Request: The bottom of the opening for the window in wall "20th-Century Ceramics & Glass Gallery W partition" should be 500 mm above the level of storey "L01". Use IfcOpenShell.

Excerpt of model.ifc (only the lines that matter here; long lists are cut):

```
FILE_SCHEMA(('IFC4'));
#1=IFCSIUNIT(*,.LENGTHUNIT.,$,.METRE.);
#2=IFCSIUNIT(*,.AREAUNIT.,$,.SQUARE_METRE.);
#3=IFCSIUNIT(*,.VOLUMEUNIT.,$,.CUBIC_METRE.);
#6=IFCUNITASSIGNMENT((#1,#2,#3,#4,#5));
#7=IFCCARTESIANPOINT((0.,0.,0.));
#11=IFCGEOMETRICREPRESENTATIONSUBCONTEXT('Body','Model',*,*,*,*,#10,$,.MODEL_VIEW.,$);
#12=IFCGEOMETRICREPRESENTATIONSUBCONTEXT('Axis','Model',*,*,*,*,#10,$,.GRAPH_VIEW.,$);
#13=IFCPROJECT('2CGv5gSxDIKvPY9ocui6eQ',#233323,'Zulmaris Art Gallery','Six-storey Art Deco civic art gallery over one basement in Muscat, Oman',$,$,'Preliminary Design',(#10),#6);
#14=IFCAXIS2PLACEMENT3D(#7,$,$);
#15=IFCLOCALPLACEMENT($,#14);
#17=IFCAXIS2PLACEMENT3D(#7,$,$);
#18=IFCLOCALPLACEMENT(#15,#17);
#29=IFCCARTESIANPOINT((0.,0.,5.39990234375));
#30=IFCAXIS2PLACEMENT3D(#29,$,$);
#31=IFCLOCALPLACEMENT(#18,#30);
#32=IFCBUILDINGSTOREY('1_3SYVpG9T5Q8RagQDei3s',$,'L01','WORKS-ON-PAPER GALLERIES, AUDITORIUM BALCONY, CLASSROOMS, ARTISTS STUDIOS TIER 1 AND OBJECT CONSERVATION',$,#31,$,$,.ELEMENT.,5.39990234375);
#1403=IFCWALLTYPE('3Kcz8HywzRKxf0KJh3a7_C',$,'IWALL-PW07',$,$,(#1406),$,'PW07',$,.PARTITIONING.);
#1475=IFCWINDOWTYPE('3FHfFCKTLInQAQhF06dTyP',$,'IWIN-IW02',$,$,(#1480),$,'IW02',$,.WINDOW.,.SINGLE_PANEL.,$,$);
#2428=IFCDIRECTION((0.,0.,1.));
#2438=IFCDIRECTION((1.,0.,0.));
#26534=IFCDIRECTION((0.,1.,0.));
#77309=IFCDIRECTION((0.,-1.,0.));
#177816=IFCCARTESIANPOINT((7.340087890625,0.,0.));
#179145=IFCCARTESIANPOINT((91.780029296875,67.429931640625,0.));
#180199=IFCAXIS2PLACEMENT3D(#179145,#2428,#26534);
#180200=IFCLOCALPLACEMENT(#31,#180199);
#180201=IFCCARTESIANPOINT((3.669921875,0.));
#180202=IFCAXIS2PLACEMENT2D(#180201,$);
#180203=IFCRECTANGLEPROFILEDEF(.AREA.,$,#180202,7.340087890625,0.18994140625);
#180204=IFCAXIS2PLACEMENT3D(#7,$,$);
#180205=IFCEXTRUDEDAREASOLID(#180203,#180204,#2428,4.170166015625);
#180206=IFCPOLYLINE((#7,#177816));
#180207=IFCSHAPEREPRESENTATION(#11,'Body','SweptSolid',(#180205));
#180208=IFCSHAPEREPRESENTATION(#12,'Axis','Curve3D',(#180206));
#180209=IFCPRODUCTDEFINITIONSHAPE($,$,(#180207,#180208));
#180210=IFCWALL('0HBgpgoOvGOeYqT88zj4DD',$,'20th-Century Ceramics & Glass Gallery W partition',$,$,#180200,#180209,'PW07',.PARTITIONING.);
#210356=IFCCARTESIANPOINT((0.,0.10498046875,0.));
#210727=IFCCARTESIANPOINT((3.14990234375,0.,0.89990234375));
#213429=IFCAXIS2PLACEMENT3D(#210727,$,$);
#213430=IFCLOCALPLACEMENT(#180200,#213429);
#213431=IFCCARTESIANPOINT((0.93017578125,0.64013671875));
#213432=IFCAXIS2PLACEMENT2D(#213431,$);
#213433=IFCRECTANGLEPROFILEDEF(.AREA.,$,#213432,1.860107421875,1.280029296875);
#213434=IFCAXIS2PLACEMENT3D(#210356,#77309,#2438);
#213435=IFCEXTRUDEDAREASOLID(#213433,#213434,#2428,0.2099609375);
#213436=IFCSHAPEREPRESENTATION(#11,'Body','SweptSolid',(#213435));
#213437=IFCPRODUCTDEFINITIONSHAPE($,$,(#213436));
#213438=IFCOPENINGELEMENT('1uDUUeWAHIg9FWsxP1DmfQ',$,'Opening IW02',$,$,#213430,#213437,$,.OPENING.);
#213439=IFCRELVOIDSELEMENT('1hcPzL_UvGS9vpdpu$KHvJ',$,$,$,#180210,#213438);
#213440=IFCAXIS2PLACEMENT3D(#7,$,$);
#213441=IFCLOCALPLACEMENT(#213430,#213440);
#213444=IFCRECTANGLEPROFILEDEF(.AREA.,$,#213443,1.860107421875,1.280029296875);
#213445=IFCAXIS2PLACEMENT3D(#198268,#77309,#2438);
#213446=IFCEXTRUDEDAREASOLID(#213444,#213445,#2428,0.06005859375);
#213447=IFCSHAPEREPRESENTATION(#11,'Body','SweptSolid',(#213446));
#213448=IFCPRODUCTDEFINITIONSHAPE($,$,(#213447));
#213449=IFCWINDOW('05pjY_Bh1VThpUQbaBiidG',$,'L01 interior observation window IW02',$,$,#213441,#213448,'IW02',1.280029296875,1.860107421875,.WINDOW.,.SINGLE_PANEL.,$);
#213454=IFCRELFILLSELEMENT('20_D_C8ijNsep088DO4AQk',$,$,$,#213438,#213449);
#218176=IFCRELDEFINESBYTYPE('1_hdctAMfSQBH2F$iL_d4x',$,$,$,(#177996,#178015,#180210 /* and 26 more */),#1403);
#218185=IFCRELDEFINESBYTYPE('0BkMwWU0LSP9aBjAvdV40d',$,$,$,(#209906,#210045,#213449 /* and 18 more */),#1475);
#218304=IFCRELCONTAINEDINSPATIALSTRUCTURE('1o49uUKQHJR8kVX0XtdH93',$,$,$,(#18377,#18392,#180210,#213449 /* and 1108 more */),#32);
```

```python
import numpy as np
import ifcopenshell
import ifcopenshell.api.geometry
import ifcopenshell.geom
import ifcopenshell.util.element
import ifcopenshell.util.placement
import ifcopenshell.util.shape
import ifcopenshell.util.unit

model = ifcopenshell.open("model.ifc")
unit_scale = ifcopenshell.util.unit.calculate_unit_scale(model)

window = model.by_guid("05pjY_Bh1VThpUQbaBiidG")
opening = window.FillsVoids[0].RelatingOpeningElement
storey = ifcopenshell.util.element.get_container(window, ifc_class="IfcBuildingStorey")
level = ifcopenshell.util.placement.get_local_placement(storey.ObjectPlacement)[2, 3]

# The opening's origin need not be at the sill, so measure its lowest point.
shape = ifcopenshell.geom.create_shape(ifcopenshell.geom.settings(), opening)
bottom = ifcopenshell.util.shape.get_shape_bottom_elevation(shape, shape.geometry) / unit_scale
dz = level + 0.5 / unit_scale - bottom

shift = np.array([0.0, 0.0, dz])
# The window is placed relative to its opening, so it follows when the opening moves.
matrix = ifcopenshell.util.placement.get_local_placement(opening.ObjectPlacement)
matrix[:3, 3] += shift
ifcopenshell.api.geometry.edit_object_placement(
    model, product=opening, matrix=matrix, is_si=False, should_transform_children=True
)

print(f"moved by {dz * unit_scale:+.3f} m")

model.write("model_edited.ifc")
```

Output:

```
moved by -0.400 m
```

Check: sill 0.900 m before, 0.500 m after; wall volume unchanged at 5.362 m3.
